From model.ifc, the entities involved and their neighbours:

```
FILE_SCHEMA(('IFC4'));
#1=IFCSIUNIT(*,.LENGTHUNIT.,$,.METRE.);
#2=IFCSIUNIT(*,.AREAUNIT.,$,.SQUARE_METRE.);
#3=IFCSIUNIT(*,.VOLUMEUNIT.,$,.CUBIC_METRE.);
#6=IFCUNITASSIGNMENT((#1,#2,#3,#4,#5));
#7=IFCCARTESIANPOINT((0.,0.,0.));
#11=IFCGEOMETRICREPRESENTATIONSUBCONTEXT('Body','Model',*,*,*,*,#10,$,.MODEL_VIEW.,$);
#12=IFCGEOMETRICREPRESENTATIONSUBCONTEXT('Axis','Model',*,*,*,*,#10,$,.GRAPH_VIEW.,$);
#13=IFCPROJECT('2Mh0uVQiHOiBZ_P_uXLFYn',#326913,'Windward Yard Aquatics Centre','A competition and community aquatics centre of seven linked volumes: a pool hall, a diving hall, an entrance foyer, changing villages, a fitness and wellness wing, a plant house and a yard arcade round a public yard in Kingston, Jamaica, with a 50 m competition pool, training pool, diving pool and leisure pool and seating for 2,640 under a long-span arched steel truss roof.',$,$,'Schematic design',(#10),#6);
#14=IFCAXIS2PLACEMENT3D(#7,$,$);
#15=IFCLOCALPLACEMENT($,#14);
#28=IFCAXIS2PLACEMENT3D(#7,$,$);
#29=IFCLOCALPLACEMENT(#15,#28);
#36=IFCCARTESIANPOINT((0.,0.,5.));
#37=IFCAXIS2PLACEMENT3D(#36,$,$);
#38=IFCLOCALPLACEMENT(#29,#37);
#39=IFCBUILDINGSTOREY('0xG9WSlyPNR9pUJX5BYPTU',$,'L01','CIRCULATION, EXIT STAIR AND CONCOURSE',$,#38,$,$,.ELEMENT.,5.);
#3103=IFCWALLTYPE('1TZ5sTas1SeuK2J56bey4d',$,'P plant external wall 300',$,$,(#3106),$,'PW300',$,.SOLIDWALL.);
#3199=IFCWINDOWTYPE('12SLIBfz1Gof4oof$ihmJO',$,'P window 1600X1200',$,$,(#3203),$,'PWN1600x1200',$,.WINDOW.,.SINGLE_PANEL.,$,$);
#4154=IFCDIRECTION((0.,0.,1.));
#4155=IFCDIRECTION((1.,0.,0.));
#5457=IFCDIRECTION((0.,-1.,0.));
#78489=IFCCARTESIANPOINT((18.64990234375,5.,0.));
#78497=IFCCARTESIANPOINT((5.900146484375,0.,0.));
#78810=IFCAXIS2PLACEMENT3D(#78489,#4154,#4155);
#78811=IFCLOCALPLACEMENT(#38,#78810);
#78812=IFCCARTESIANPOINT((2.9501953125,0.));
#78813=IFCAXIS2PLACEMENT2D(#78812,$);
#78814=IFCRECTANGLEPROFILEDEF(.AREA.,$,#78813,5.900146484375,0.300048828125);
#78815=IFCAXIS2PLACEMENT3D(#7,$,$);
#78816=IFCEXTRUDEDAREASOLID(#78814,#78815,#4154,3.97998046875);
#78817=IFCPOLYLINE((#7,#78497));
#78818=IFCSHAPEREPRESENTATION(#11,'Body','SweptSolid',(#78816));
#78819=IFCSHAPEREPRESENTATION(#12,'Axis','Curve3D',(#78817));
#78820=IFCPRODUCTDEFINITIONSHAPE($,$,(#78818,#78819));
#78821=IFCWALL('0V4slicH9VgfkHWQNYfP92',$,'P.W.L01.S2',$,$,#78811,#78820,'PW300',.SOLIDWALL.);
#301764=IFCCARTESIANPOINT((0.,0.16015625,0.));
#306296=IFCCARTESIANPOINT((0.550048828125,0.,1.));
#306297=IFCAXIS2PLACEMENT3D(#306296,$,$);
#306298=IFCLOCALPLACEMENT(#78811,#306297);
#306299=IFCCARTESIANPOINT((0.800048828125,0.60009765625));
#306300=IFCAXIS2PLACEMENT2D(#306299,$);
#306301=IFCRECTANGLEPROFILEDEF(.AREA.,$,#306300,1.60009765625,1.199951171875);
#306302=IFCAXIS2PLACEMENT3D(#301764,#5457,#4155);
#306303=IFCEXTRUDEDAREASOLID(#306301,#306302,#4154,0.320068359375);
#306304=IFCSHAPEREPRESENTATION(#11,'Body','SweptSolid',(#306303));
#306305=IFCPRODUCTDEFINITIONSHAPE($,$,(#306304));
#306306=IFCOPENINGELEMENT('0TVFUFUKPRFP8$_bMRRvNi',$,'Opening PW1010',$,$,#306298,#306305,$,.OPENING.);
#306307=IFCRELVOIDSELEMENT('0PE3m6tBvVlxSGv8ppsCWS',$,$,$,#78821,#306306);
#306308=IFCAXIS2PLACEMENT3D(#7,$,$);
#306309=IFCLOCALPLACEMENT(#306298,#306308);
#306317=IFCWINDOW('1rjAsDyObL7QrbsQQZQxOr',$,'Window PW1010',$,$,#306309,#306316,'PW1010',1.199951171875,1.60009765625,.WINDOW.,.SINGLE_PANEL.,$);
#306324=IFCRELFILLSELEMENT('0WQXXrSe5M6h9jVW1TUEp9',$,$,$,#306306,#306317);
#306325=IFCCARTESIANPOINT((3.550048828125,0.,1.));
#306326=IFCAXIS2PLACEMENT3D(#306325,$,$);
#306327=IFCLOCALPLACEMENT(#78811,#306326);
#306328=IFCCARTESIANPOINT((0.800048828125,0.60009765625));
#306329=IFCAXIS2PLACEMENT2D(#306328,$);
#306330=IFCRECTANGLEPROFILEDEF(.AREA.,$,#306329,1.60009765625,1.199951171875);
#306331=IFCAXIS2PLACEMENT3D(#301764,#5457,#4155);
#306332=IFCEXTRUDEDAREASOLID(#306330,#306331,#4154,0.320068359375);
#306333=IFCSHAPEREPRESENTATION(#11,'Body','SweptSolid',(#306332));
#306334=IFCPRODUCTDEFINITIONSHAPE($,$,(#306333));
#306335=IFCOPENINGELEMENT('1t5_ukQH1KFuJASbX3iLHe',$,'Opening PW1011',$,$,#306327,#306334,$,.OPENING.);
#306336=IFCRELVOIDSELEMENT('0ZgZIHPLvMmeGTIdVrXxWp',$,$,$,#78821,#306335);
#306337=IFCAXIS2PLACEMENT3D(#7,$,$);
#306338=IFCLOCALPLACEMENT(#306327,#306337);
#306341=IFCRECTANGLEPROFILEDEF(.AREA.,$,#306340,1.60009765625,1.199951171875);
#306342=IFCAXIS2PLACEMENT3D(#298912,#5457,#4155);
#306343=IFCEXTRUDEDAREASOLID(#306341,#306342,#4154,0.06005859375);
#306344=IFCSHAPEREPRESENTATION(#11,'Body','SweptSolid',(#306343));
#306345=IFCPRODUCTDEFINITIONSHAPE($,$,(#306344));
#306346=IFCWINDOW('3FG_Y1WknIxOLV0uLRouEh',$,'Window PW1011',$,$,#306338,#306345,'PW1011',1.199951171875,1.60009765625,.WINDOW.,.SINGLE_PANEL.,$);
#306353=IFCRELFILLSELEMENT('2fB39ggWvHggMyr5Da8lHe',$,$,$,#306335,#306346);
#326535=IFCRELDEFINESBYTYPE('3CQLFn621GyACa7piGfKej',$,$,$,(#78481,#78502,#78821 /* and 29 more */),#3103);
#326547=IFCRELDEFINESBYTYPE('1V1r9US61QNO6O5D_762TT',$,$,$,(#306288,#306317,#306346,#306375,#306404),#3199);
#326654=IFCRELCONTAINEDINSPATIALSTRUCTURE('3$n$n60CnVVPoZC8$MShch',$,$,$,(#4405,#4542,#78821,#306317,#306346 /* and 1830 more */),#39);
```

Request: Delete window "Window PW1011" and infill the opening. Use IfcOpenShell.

```python
import ifcopenshell
import ifcopenshell.api.feature
import ifcopenshell.api.root
import ifcopenshell.geom
import ifcopenshell.util.shape

model = ifcopenshell.open("model.ifc")
settings = ifcopenshell.geom.settings()


def volume(element):
    """Net volume in cubic metres, openings subtracted."""
    shape = ifcopenshell.geom.create_shape(settings, element)
    return ifcopenshell.util.shape.get_volume(shape.geometry)


window = model.by_id(306346)
opening = window.FillsVoids[0].RelatingOpeningElement
wall = opening.VoidsElements[0].RelatingBuildingElement
before = volume(wall)

ifcopenshell.api.root.remove_product(model, product=window)
ifcopenshell.api.feature.remove_feature(model, feature=opening)

after = volume(wall)

print(f"wall volume {before:.3f} -> {after:.3f} m3")

model.write("model_updated.ifc")
```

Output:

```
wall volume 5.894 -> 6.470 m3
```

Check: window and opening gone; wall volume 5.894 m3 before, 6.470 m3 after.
